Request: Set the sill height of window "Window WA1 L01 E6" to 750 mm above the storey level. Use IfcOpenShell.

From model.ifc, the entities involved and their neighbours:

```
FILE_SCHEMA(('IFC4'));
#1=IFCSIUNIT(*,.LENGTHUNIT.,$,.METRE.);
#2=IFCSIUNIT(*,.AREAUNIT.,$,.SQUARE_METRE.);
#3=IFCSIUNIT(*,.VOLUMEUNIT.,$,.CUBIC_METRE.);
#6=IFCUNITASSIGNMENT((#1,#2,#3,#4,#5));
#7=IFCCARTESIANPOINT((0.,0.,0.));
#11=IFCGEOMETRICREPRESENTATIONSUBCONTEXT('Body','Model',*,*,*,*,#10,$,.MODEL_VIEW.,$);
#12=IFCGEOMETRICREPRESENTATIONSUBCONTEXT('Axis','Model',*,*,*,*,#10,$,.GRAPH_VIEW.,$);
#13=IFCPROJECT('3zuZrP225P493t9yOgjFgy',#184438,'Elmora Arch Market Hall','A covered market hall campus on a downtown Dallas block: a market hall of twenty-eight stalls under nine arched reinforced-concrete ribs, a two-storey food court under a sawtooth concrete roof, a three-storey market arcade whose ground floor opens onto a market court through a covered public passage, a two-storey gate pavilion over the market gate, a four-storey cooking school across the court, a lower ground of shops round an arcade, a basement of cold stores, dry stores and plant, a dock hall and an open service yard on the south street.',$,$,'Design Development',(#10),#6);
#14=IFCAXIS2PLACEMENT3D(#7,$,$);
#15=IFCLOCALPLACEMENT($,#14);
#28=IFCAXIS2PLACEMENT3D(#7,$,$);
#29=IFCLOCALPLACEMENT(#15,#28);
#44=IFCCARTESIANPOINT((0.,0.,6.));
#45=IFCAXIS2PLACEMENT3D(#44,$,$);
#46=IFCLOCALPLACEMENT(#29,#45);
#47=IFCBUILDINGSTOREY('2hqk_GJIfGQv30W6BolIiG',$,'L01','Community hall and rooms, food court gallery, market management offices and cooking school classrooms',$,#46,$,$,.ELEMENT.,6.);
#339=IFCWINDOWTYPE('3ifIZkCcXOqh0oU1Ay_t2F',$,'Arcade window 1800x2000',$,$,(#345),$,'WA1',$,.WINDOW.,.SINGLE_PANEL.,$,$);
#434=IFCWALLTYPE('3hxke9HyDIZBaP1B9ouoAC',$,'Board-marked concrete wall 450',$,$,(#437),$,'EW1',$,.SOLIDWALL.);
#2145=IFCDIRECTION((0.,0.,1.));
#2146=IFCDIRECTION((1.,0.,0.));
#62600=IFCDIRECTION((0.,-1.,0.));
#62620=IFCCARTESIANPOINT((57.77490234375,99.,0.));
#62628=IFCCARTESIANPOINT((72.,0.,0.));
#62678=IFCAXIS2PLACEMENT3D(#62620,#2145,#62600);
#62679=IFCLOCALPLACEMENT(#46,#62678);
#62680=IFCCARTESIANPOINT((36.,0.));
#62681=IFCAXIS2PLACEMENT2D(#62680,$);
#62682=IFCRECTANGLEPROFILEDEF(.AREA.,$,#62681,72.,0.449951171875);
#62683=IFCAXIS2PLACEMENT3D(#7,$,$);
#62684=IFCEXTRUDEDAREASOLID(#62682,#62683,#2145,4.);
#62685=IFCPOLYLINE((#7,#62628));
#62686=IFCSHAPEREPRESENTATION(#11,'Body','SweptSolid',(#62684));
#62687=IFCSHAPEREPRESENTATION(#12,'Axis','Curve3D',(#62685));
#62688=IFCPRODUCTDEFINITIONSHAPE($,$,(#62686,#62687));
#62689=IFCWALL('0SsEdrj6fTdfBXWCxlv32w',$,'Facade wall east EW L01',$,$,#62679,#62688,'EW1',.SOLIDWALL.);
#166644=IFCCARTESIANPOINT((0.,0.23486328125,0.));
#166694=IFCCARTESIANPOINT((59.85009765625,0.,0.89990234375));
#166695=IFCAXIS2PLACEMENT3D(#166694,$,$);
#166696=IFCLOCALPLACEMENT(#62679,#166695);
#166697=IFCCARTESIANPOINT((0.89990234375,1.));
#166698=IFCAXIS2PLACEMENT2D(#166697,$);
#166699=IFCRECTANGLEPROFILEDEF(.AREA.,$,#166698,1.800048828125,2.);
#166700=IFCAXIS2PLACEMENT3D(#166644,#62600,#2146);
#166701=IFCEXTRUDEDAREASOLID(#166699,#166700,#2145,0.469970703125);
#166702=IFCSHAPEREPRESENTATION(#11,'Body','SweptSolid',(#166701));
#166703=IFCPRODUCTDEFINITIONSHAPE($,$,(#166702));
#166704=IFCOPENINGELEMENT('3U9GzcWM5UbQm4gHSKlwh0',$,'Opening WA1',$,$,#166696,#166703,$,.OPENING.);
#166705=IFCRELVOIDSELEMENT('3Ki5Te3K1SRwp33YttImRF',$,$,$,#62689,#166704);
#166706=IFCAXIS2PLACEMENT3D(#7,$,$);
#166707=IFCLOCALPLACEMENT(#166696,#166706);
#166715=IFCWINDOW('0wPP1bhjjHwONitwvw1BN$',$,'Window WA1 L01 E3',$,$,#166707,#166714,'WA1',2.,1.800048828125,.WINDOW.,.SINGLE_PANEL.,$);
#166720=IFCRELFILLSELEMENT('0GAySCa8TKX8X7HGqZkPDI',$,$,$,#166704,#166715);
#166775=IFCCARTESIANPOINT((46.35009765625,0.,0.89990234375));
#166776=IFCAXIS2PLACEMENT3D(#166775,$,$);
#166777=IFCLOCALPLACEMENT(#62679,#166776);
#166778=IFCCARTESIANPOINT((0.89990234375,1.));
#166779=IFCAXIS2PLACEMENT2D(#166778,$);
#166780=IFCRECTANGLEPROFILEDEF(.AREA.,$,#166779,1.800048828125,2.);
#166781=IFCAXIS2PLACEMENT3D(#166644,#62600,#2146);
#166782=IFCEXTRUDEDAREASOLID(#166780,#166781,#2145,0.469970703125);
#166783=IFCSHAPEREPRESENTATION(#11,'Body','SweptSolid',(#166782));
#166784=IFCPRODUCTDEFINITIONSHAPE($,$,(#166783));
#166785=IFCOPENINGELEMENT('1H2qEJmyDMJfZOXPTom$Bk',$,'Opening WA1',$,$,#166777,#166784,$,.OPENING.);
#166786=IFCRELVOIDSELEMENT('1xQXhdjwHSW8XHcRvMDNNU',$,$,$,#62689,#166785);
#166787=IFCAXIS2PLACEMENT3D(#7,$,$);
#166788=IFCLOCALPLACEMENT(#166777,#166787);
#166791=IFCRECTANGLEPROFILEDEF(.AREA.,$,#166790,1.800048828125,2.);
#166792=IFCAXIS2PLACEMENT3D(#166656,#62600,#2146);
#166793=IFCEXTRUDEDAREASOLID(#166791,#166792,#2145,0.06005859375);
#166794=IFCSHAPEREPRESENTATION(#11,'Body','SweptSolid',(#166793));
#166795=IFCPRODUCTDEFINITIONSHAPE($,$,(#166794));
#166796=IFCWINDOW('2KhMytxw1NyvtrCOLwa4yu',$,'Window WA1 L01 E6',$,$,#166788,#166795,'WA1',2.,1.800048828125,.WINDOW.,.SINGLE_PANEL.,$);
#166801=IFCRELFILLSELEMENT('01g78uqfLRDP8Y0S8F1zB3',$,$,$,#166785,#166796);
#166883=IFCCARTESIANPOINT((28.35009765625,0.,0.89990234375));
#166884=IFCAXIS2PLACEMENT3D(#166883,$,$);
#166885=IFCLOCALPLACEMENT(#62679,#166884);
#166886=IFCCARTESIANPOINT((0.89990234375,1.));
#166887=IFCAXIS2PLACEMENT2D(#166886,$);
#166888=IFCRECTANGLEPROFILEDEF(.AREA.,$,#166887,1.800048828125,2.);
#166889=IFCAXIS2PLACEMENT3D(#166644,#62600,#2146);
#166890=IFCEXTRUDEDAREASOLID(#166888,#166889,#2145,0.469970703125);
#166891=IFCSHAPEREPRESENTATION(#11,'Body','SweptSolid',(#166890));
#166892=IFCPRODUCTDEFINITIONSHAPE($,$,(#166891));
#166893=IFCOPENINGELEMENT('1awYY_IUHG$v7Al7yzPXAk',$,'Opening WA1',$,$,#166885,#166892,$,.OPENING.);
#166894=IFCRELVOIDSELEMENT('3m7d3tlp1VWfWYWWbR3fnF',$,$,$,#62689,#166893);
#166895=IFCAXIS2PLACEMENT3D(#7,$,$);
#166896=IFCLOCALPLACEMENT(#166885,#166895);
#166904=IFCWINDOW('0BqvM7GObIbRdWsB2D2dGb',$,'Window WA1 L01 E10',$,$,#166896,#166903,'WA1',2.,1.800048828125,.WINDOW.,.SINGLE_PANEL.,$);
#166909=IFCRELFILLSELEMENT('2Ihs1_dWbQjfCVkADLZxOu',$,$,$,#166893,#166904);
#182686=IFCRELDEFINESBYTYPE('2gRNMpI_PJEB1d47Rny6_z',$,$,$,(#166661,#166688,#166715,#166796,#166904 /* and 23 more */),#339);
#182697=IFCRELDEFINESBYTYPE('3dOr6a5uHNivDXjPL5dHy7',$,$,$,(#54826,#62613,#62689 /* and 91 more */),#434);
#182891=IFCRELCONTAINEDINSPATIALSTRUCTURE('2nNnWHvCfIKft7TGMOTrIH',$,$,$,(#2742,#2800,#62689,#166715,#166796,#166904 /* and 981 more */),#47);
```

```python
import numpy as np
import ifcopenshell
import ifcopenshell.api.geometry
import ifcopenshell.geom
import ifcopenshell.util.element
import ifcopenshell.util.placement
import ifcopenshell.util.shape
import ifcopenshell.util.unit

model = ifcopenshell.open("model.ifc")
unit_scale = ifcopenshell.util.unit.calculate_unit_scale(model)

window = model.by_id(166796)
opening = window.FillsVoids[0].RelatingOpeningElement
storey = ifcopenshell.util.element.get_container(window, ifc_class="IfcBuildingStorey")
level = ifcopenshell.util.placement.get_local_placement(storey.ObjectPlacement)[2, 3]

# The opening's origin need not be at the sill, so measure its lowest point.
shape = ifcopenshell.geom.create_shape(ifcopenshell.geom.settings(), opening)
bottom = ifcopenshell.util.shape.get_shape_bottom_elevation(shape, shape.geometry) / unit_scale
dz = level + 0.75 / unit_scale - bottom

shift = np.array([0.0, 0.0, dz])
# The window is placed relative to its opening, so it follows when the opening moves.
matrix = ifcopenshell.util.placement.get_local_placement(opening.ObjectPlacement)
matrix[:3, 3] += shift
ifcopenshell.api.geometry.edit_object_placement(
    model, product=opening, matrix=matrix, is_si=False, should_transform_children=True
)

print(f"moved by {dz * unit_scale:+.3f} m")

model.write("model_updated.ifc")
```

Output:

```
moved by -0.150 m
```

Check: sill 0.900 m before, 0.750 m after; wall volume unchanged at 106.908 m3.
